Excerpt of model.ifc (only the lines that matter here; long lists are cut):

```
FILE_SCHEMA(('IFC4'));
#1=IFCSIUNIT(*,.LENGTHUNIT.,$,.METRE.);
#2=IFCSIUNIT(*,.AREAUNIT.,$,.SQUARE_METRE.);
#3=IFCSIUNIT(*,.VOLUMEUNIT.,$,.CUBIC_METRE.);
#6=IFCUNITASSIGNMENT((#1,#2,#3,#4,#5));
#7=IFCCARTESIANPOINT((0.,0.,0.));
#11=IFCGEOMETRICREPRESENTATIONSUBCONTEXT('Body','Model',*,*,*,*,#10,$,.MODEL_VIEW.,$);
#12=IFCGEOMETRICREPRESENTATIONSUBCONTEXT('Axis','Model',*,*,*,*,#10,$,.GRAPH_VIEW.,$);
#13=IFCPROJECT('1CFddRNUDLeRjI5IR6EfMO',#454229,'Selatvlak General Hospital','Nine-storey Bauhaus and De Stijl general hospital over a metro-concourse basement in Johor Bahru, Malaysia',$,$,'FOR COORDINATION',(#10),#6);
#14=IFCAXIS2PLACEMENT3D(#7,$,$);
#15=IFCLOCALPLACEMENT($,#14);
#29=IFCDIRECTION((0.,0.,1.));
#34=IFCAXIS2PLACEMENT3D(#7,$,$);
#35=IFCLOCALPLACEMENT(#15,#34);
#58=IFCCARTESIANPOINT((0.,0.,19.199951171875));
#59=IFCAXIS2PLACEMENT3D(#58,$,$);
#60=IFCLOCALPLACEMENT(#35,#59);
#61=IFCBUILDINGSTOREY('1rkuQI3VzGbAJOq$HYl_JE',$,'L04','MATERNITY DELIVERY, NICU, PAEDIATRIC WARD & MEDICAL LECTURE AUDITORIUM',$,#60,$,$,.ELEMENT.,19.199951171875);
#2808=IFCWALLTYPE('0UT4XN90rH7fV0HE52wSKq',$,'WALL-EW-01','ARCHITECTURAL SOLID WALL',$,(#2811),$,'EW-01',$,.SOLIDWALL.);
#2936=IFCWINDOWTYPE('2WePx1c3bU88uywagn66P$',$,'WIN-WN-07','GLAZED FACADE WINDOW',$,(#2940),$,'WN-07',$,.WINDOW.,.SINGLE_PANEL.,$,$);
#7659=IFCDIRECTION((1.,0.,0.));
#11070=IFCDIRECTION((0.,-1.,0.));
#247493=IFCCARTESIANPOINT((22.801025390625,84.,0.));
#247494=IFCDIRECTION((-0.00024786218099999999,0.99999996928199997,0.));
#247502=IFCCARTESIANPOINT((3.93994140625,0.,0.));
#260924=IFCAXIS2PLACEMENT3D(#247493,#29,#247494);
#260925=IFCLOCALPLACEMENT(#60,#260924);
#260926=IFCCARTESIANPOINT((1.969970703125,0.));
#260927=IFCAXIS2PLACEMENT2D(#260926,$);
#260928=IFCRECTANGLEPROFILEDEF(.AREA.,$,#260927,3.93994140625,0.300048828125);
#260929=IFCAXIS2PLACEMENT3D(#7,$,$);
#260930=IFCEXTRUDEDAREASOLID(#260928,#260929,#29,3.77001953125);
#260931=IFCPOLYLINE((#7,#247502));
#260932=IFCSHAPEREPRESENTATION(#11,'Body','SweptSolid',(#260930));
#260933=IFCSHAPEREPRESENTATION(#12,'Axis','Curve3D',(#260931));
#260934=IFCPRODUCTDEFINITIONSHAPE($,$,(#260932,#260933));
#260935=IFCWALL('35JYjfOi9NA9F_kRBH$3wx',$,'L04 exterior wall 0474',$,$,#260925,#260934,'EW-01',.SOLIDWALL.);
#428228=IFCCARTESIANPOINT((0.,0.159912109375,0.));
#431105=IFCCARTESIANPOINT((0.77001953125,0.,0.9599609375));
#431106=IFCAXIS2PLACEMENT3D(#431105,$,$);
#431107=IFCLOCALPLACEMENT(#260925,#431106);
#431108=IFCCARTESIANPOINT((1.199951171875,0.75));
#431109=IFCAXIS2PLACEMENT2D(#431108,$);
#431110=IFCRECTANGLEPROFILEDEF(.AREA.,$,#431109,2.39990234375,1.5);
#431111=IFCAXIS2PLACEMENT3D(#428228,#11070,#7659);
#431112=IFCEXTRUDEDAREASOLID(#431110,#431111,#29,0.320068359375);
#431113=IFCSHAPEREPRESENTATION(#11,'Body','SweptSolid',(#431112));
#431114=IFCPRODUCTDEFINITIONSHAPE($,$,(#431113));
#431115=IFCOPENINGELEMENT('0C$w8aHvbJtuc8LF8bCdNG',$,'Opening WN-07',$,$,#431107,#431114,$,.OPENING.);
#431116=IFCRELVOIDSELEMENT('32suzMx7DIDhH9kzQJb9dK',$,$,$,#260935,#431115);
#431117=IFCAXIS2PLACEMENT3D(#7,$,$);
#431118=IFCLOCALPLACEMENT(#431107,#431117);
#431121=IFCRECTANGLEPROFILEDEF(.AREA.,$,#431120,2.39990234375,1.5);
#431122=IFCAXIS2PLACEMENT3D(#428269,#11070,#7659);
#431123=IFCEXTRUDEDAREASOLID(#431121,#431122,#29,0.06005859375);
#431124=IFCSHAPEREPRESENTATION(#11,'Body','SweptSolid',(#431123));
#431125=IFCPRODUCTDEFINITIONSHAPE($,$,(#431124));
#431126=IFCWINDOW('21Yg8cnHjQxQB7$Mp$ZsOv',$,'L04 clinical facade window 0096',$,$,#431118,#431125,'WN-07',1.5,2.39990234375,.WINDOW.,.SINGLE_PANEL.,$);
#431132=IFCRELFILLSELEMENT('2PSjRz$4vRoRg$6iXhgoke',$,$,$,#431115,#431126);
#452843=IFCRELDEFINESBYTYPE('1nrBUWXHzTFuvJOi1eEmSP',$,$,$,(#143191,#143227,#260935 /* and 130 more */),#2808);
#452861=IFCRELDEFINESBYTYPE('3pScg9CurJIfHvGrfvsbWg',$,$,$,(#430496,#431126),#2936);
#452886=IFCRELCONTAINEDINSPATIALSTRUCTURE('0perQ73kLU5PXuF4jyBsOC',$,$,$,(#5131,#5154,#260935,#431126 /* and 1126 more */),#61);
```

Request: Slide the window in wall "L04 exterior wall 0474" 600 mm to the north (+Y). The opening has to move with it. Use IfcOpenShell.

```python
import ifcopenshell
import ifcopenshell.api.geometry
import ifcopenshell.util.placement

model = ifcopenshell.open("model.ifc")

window = model.by_guid("21Yg8cnHjQxQB7$Mp$ZsOv")
opening = window.FillsVoids[0].RelatingOpeningElement
wall = opening.VoidsElements[0].RelatingBuildingElement

wall_matrix = ifcopenshell.util.placement.get_local_placement(wall.ObjectPlacement)
shift = wall_matrix[:3, 0] * 0.6
before = ifcopenshell.util.placement.get_local_placement(window.ObjectPlacement)[:3, 3].copy()

# The window is placed relative to its opening, so it follows when the opening moves.
matrix = ifcopenshell.util.placement.get_local_placement(opening.ObjectPlacement)
matrix[:3, 3] += shift
ifcopenshell.api.geometry.edit_object_placement(
    model, product=opening, matrix=matrix, is_si=False, should_transform_children=True
)

after = ifcopenshell.util.placement.get_local_placement(window.ObjectPlacement)[:3, 3]
print("window moved by", (after - before).round(3) + 0.0)

model.write("model-out.ifc")
```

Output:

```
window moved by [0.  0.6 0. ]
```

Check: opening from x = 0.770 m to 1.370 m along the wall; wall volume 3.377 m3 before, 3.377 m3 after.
